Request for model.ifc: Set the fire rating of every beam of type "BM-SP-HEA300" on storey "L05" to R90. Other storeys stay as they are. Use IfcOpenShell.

First a look at what the model holds.

```python
import ifcopenshell
import ifcopenshell.util.element

model = ifcopenshell.open("model.ifc")
print(model.schema)
storey = next(s for s in model.by_type("IfcBuildingStorey") if s.Name == "L05")
beams = [e for e in ifcopenshell.util.element.get_decomposition(storey) if e.is_a("IfcBeam")]
seen = {}
for e in beams:
    element_type = ifcopenshell.util.element.get_type(e)
    key = (element_type.Name if element_type != e and element_type else None, ifcopenshell.util.element.get_pset(e, "Pset_BeamCommon", "FireRating"))
    seen[key] = seen.get(key, 0) + 1
for (name, value), count in sorted(seen.items(), key=str):
    print(count, "x", name, "|", value)
```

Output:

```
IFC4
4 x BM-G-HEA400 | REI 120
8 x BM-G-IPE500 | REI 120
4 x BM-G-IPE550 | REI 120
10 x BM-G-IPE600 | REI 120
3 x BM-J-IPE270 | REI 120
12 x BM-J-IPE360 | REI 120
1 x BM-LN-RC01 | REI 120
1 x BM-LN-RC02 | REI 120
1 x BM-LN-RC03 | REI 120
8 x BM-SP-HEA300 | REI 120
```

```python
import ifcopenshell
import ifcopenshell.api.pset
import ifcopenshell.util.element

model = ifcopenshell.open("model.ifc")

storey = next(s for s in model.by_type("IfcBuildingStorey") if s.Name == "L05")
beams = [e for e in ifcopenshell.util.element.get_decomposition(storey) if e.is_a("IfcBeam")]

count = 0
for e in beams:
    element_type = ifcopenshell.util.element.get_type(e)
    if element_type in (None, e) or element_type.Name != "BM-SP-HEA300":
        continue
    # add_pset returns the element's existing set when there is one.
    pset = ifcopenshell.api.pset.add_pset(model, product=e, name="Pset_BeamCommon")
    ifcopenshell.api.pset.edit_pset(model, pset=pset, properties={"FireRating": "R90"})
    count += 1

print(count, "beams updated")

model.write("model-out.ifc")
```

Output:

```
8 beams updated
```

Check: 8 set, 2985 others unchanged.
